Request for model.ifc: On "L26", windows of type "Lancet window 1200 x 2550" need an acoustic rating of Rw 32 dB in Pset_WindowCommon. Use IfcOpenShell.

First a look at what the model holds.

```python
import ifcopenshell
import ifcopenshell.util.element

model = ifcopenshell.open("model.ifc")
print(model.schema)
storey = next(s for s in model.by_type("IfcBuildingStorey") if s.Name == "L26")
windows = [e for e in ifcopenshell.util.element.get_decomposition(storey) if e.is_a("IfcWindow")]
seen = {}
for e in windows:
    element_type = ifcopenshell.util.element.get_type(e)
    key = (element_type.Name if element_type != e and element_type else None, ifcopenshell.util.element.get_pset(e, "Pset_WindowCommon", "AcousticRating"))
    seen[key] = seen.get(key, 0) + 1
for (name, value), count in sorted(seen.items(), key=str):
    print(count, "x", name, "|", value)
```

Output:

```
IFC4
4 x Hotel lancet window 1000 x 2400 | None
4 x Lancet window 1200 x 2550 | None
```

```python
import ifcopenshell
import ifcopenshell.api.pset
import ifcopenshell.util.element

model = ifcopenshell.open("model.ifc")

storey = next(s for s in model.by_type("IfcBuildingStorey") if s.Name == "L26")
windows = [e for e in ifcopenshell.util.element.get_decomposition(storey) if e.is_a("IfcWindow")]

count = 0
for e in windows:
    element_type = ifcopenshell.util.element.get_type(e)
    if element_type in (None, e) or element_type.Name != "Lancet window 1200 x 2550":
        continue
    found = ifcopenshell.util.element.get_pset(e, "Pset_WindowCommon", should_inherit=False)
    if found:
        pset = model.by_id(found["id"])
        if len(ifcopenshell.util.element.get_elements_by_pset(pset)) > 1:
            pset = ifcopenshell.api.pset.unshare_pset(model, products=[e], pset=pset)[0]
    else:
        pset = ifcopenshell.api.pset.add_pset(model, product=e, name="Pset_WindowCommon")
    ifcopenshell.api.pset.edit_pset(model, pset=pset, properties={"AcousticRating": "Rw 32 dB"})
    count += 1

print(count, "windows updated")

model.write("model_updated.ifc")
```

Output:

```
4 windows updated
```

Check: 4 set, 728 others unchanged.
